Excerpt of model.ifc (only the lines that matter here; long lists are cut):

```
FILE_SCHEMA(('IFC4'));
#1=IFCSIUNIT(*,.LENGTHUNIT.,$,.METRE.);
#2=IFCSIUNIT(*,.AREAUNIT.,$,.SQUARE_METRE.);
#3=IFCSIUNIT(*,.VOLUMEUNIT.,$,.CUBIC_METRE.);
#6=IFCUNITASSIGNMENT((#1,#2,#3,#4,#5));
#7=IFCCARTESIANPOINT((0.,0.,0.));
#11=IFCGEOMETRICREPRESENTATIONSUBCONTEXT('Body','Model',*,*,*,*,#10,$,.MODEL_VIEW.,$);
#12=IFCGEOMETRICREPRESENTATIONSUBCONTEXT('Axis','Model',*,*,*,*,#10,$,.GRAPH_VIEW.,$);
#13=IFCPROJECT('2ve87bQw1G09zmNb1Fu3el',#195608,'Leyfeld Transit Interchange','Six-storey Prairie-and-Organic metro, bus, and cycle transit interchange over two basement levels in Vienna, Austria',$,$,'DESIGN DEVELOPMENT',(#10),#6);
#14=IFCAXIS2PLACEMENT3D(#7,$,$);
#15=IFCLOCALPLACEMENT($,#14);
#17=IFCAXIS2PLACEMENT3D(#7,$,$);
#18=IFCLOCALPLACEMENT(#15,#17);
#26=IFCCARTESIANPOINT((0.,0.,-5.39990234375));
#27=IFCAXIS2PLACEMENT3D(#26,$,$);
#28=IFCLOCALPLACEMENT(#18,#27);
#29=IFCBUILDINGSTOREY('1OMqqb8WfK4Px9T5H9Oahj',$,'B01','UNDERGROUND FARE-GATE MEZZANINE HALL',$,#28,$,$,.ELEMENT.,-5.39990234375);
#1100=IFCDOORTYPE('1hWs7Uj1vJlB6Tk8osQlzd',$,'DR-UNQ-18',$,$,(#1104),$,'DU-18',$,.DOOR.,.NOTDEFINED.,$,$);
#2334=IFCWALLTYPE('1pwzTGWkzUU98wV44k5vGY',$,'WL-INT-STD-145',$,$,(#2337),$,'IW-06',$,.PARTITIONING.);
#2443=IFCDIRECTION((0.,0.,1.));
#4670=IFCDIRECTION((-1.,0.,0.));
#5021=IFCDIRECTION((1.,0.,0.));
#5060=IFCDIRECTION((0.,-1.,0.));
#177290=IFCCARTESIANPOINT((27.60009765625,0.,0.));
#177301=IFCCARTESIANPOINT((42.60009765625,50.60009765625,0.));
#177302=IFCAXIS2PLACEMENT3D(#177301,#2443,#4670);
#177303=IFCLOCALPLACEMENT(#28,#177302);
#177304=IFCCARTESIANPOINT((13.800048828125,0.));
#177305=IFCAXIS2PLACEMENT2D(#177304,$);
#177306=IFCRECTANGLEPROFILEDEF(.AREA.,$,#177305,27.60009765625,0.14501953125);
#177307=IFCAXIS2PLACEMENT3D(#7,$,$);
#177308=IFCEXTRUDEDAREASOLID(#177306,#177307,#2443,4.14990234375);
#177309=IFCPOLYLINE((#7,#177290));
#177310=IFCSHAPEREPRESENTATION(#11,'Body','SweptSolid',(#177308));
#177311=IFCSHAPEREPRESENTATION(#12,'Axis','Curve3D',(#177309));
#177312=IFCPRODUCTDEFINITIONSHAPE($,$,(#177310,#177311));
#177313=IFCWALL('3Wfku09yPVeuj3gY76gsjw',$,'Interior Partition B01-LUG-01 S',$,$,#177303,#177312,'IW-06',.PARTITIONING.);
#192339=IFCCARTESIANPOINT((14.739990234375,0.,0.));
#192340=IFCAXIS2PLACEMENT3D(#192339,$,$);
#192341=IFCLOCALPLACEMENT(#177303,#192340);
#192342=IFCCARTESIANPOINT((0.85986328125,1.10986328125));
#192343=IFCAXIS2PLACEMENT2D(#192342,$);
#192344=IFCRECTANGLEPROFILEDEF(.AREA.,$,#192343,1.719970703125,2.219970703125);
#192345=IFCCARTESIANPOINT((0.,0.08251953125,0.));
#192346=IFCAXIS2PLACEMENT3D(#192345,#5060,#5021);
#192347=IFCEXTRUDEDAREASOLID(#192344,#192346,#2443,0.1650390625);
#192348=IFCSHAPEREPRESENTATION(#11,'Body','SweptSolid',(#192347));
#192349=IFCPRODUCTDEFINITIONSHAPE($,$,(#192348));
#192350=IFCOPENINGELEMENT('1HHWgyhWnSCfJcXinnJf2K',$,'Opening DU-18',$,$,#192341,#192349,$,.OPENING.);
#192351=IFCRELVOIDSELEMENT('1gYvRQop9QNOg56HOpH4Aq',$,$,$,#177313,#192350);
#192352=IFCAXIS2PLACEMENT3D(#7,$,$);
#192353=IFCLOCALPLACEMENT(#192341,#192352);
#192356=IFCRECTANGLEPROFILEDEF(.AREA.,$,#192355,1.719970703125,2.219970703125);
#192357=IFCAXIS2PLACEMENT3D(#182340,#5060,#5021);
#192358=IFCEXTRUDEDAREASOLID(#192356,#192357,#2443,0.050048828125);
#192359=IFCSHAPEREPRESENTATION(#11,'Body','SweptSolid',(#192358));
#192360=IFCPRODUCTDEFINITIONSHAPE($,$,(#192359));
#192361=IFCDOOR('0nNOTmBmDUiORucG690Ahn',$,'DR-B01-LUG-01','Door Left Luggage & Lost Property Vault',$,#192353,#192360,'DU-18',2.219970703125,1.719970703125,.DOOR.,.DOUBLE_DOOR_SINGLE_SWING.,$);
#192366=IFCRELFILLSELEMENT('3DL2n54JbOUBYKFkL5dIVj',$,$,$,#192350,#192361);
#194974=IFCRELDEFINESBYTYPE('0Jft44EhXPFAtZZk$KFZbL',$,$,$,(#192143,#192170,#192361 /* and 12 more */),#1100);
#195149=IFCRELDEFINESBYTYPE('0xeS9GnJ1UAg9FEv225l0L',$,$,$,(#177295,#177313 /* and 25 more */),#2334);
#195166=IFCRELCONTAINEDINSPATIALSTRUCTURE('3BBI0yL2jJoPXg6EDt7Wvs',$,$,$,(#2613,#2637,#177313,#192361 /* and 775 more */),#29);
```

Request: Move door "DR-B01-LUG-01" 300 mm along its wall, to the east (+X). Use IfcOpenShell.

```python
import ifcopenshell
import ifcopenshell.api.geometry
import ifcopenshell.util.placement

model = ifcopenshell.open("model.ifc")

door = model.by_guid("0nNOTmBmDUiORucG690Ahn")
opening = door.FillsVoids[0].RelatingOpeningElement
wall = opening.VoidsElements[0].RelatingBuildingElement

wall_matrix = ifcopenshell.util.placement.get_local_placement(wall.ObjectPlacement)
shift = wall_matrix[:3, 0] * -0.3
before = ifcopenshell.util.placement.get_local_placement(door.ObjectPlacement)[:3, 3].copy()

# The door is placed relative to its opening, so it follows when the opening moves.
matrix = ifcopenshell.util.placement.get_local_placement(opening.ObjectPlacement)
matrix[:3, 3] += shift
ifcopenshell.api.geometry.edit_object_placement(
    model, product=opening, matrix=matrix, is_si=False, should_transform_children=True
)

after = ifcopenshell.util.placement.get_local_placement(door.ObjectPlacement)[:3, 3]
print("door moved by", (after - before).round(3) + 0.0)

model.write("model_edited.ifc")
```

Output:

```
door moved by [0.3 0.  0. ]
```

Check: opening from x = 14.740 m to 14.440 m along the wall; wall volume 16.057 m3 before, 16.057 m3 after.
